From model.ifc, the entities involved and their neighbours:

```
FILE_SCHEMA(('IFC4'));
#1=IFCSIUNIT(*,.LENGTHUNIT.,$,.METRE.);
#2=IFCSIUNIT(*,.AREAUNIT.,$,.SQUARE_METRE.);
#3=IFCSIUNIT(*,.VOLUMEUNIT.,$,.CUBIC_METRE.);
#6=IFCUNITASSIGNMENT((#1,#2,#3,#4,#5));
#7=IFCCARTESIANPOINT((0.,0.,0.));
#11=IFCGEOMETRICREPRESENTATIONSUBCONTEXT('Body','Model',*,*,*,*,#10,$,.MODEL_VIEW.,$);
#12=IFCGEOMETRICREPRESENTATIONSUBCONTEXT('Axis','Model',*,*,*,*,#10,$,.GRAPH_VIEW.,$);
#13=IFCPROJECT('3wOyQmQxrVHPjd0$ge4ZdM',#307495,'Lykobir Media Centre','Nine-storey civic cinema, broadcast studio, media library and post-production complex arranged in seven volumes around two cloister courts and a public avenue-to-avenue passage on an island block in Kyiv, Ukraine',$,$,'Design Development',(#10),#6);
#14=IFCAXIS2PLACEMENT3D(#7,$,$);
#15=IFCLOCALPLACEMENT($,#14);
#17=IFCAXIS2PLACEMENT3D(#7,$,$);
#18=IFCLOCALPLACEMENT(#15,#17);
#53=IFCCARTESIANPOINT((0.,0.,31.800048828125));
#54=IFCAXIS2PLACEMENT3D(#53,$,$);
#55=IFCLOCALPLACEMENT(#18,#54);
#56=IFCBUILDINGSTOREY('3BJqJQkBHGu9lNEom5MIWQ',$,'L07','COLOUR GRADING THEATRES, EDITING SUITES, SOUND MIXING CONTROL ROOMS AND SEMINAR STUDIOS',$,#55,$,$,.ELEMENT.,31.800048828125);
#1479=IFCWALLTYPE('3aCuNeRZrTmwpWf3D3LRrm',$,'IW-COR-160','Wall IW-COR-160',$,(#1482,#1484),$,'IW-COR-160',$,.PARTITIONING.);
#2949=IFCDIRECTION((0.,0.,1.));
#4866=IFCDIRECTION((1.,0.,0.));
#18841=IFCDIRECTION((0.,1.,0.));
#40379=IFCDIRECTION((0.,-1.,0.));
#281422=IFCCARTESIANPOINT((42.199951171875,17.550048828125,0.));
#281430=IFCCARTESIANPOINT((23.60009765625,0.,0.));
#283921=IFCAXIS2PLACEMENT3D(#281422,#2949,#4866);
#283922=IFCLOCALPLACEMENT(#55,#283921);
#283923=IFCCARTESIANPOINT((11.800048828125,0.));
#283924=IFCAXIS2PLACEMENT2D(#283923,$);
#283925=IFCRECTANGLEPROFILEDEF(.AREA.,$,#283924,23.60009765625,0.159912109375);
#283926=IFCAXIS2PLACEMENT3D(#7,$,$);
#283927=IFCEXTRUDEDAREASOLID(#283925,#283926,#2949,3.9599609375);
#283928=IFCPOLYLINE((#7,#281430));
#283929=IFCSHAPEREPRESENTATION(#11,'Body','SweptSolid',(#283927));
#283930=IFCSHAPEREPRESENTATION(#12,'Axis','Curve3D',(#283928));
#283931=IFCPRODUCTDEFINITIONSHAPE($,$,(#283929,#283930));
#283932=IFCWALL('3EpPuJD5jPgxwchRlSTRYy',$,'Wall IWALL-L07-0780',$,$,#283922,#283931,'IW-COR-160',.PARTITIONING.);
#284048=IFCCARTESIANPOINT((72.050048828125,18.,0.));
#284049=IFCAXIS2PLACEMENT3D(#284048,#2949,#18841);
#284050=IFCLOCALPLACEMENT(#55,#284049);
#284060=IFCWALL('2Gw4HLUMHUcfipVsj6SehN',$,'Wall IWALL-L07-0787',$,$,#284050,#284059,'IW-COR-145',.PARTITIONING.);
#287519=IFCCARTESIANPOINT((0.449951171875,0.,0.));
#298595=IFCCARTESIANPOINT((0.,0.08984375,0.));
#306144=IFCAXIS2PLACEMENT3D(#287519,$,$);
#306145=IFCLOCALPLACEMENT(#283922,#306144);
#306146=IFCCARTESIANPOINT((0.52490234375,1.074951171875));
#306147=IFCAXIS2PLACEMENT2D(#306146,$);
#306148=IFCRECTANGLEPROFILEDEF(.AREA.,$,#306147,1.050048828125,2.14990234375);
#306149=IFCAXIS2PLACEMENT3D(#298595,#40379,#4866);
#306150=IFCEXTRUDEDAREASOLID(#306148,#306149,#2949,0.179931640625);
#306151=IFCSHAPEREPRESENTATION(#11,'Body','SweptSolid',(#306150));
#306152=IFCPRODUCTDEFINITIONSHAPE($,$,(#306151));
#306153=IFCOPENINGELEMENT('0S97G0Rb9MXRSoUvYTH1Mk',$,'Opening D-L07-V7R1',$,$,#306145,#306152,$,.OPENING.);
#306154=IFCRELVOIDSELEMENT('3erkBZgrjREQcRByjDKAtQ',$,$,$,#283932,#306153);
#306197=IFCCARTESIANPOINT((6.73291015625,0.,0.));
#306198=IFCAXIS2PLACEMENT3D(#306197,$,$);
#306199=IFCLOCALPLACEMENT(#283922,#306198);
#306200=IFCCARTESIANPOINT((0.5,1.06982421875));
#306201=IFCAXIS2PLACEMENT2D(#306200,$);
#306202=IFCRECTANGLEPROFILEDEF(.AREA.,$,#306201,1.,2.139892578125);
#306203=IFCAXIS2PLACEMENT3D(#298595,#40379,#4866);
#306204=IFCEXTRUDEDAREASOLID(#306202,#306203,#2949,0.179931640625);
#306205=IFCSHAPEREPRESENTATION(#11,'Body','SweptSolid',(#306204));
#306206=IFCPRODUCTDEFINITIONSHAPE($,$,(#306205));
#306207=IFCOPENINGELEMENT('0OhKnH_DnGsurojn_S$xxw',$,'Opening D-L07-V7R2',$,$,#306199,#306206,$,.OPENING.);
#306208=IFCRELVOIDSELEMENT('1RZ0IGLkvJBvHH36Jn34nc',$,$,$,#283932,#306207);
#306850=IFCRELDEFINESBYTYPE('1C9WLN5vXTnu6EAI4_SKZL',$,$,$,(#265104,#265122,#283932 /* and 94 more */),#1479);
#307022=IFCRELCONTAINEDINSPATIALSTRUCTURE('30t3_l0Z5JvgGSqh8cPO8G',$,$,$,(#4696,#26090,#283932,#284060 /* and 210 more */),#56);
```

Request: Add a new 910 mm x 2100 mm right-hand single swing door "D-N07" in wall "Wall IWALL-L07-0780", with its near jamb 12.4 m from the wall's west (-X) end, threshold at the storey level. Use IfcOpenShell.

```python
import numpy as np
import ifcopenshell
import ifcopenshell.api.feature
import ifcopenshell.api.geometry
import ifcopenshell.api.root
import ifcopenshell.api.spatial
import ifcopenshell.geom
import ifcopenshell.util.element
import ifcopenshell.util.placement
import ifcopenshell.util.representation
import ifcopenshell.util.shape
import ifcopenshell.util.unit

model = ifcopenshell.open("model.ifc")
unit_scale = ifcopenshell.util.unit.calculate_unit_scale(model)
settings = ifcopenshell.geom.settings()


def volume(element):
    """Net volume in cubic metres, openings subtracted."""
    shape = ifcopenshell.geom.create_shape(settings, element)
    return ifcopenshell.util.shape.get_volume(shape.geometry)


wall = model.by_guid("3EpPuJD5jPgxwchRlSTRYy")
storey = ifcopenshell.util.element.get_container(wall, ifc_class="IfcBuildingStorey")
context = ifcopenshell.util.representation.get_context(model, "Model", "Body", "MODEL_VIEW")
before = volume(wall)

width, height, from_end, sill = 0.91, 2.1, 12.4, 0.0  # metres

# The wall runs along its own X axis, and the end named is its -X end.
wall_shape = ifcopenshell.geom.create_shape(settings, wall)
x, y, z = ifcopenshell.util.shape.get_vertices(wall_shape.geometry).T
start = x.min() + from_end
face, thickness = float(y.min()), float(y.max() - y.min())
wall_matrix = ifcopenshell.util.placement.get_local_placement(wall.ObjectPlacement)
level = ifcopenshell.util.placement.get_local_placement(storey.ObjectPlacement)[2, 3]


def in_wall(x, y):
    """Placement at x, y metres in the wall's axes, at sill height."""
    matrix = wall_matrix.copy()
    matrix[:, 3] = wall_matrix @ np.array([x / unit_scale, y / unit_scale, 0.0, 1.0])
    matrix[2, 3] = level + sill / unit_scale
    return matrix


# Opening: a box that overshoots both wall faces by 50 mm.
opening = ifcopenshell.api.root.create_entity(model, ifc_class="IfcOpeningElement", predefined_type="OPENING")
box = ifcopenshell.api.geometry.add_wall_representation(
    model, context=context, length=width, height=height, thickness=thickness + 0.1
)
ifcopenshell.api.geometry.assign_representation(model, product=opening, representation=box)
ifcopenshell.api.geometry.edit_object_placement(model, product=opening, matrix=in_wall(start, face - 0.05), is_si=False)
ifcopenshell.api.feature.add_feature(model, feature=opening, element=wall)

door = ifcopenshell.api.root.create_entity(model, ifc_class="IfcDoor", name="D-N07", predefined_type="DOOR")
door.OverallWidth, door.OverallHeight = width / unit_scale, height / unit_scale
door.OperationType = "SINGLE_SWING_RIGHT"
body = ifcopenshell.api.geometry.add_door_representation(
    model,
    context=context,
    overall_width=door.OverallWidth,
    overall_height=door.OverallHeight,
    operation_type="SINGLE_SWING_RIGHT",
    lining_properties={"LiningDepth": thickness / unit_scale, "ThresholdDepth": thickness / unit_scale},
)
ifcopenshell.api.geometry.assign_representation(model, product=door, representation=body)
ifcopenshell.api.spatial.assign_container(model, products=[door], relating_structure=storey)
ifcopenshell.api.feature.add_filling(model, opening=opening, element=door)

# The lining spans the wall, so the door starts at the wall face.
ifcopenshell.api.geometry.edit_object_placement(model, product=door, matrix=in_wall(start, face), is_si=False)

after = volume(wall)

print(f"wall volume {before:.3f} -> {after:.3f} m3")

model.write("model-out.ifc")
```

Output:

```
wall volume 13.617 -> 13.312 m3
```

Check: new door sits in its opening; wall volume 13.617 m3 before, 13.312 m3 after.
